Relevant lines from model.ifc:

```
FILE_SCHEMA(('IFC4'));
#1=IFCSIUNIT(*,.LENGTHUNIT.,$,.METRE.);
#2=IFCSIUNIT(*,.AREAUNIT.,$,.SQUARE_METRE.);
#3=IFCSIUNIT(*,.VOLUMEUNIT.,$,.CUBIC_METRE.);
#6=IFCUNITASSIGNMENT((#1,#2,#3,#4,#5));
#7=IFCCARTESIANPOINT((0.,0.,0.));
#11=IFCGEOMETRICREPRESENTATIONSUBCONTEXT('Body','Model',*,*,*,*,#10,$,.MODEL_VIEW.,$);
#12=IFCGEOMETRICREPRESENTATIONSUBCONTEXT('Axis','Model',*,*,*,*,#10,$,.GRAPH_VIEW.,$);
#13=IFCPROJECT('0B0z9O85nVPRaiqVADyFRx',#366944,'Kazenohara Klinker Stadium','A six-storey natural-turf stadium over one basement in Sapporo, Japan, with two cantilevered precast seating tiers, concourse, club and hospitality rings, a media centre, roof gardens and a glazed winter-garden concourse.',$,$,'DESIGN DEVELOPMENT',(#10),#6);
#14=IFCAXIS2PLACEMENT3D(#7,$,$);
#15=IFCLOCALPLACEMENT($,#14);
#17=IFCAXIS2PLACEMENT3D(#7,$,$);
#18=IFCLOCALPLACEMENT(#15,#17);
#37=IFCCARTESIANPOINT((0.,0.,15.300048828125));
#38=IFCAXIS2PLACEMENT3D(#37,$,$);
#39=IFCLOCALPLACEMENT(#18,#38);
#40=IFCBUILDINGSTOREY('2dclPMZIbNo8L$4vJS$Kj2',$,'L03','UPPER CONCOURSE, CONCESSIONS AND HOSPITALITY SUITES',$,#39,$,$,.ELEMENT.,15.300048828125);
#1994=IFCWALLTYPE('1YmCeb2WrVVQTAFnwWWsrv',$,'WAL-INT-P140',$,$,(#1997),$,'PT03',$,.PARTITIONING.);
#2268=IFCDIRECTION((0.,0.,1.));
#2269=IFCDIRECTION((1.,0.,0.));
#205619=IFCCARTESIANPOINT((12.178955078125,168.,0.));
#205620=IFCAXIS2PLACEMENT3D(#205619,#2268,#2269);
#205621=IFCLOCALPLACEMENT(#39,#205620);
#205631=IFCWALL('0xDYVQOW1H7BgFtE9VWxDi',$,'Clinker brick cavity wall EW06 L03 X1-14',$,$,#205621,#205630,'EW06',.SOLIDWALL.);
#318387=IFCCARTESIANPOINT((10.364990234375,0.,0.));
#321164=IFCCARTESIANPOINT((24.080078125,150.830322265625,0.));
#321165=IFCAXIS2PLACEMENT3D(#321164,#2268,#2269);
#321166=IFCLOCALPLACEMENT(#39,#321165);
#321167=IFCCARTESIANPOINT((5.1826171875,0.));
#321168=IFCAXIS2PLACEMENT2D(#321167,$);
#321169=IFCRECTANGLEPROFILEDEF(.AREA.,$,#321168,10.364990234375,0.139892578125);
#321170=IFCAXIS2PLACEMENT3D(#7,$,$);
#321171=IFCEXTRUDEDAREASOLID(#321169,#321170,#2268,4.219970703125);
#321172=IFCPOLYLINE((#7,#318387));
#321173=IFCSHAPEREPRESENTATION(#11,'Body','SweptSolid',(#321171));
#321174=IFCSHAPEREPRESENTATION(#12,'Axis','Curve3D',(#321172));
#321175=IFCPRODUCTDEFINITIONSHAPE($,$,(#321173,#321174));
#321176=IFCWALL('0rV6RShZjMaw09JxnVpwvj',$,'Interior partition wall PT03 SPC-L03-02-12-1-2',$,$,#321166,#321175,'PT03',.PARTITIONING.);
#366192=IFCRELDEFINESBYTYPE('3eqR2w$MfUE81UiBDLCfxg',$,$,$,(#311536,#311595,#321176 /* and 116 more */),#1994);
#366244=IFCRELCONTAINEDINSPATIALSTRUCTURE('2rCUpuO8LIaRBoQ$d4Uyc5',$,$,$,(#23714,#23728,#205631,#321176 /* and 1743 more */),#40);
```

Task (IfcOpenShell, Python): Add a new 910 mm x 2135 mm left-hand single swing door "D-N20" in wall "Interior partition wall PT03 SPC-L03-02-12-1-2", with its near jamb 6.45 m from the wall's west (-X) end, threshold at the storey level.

```python
import numpy as np
import ifcopenshell
import ifcopenshell.api.feature
import ifcopenshell.api.geometry
import ifcopenshell.api.root
import ifcopenshell.api.spatial
import ifcopenshell.geom
import ifcopenshell.util.element
import ifcopenshell.util.placement
import ifcopenshell.util.representation
import ifcopenshell.util.shape
import ifcopenshell.util.unit

model = ifcopenshell.open("model.ifc")
unit_scale = ifcopenshell.util.unit.calculate_unit_scale(model)
settings = ifcopenshell.geom.settings()


def volume(element):
    """Net volume in cubic metres, openings subtracted."""
    shape = ifcopenshell.geom.create_shape(settings, element)
    return ifcopenshell.util.shape.get_volume(shape.geometry)


wall = model.by_guid("0rV6RShZjMaw09JxnVpwvj")
storey = ifcopenshell.util.element.get_container(wall, ifc_class="IfcBuildingStorey")
context = ifcopenshell.util.representation.get_context(model, "Model", "Body", "MODEL_VIEW")
before = volume(wall)

width, height, from_end, sill = 0.91, 2.135, 6.45, 0.0  # metres

# The wall runs along its own X axis, and the end named is its -X end.
wall_shape = ifcopenshell.geom.create_shape(settings, wall)
x, y, z = ifcopenshell.util.shape.get_vertices(wall_shape.geometry).T
start = x.min() + from_end
face, thickness = float(y.min()), float(y.max() - y.min())
wall_matrix = ifcopenshell.util.placement.get_local_placement(wall.ObjectPlacement)
level = ifcopenshell.util.placement.get_local_placement(storey.ObjectPlacement)[2, 3]


def in_wall(x, y):
    """Placement at x, y metres in the wall's axes, at sill height."""
    matrix = wall_matrix.copy()
    matrix[:, 3] = wall_matrix @ np.array([x / unit_scale, y / unit_scale, 0.0, 1.0])
    matrix[2, 3] = level + sill / unit_scale
    return matrix


# Opening: a box that overshoots both wall faces by 50 mm.
opening = ifcopenshell.api.root.create_entity(model, ifc_class="IfcOpeningElement", predefined_type="OPENING")
box = ifcopenshell.api.geometry.add_wall_representation(
    model, context=context, length=width, height=height, thickness=thickness + 0.1
)
ifcopenshell.api.geometry.assign_representation(model, product=opening, representation=box)
ifcopenshell.api.geometry.edit_object_placement(model, product=opening, matrix=in_wall(start, face - 0.05), is_si=False)
ifcopenshell.api.feature.add_feature(model, feature=opening, element=wall)

door = ifcopenshell.api.root.create_entity(model, ifc_class="IfcDoor", name="D-N20", predefined_type="DOOR")
door.OverallWidth, door.OverallHeight = width / unit_scale, height / unit_scale
door.OperationType = "SINGLE_SWING_LEFT"
body = ifcopenshell.api.geometry.add_door_representation(
    model,
    context=context,
    overall_width=door.OverallWidth,
    overall_height=door.OverallHeight,
    operation_type="SINGLE_SWING_LEFT",
    lining_properties={"LiningDepth": thickness / unit_scale, "ThresholdDepth": thickness / unit_scale},
)
ifcopenshell.api.geometry.assign_representation(model, product=door, representation=body)
ifcopenshell.api.spatial.assign_container(model, products=[door], relating_structure=storey)
ifcopenshell.api.feature.add_filling(model, opening=opening, element=door)

# The lining spans the wall, so the door starts at the wall face.
ifcopenshell.api.geometry.edit_object_placement(model, product=door, matrix=in_wall(start, face), is_si=False)

after = volume(wall)

print(f"wall volume {before:.3f} -> {after:.3f} m3")

model.write("model-out.ifc")
```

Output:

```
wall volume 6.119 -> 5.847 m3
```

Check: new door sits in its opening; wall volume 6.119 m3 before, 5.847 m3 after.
